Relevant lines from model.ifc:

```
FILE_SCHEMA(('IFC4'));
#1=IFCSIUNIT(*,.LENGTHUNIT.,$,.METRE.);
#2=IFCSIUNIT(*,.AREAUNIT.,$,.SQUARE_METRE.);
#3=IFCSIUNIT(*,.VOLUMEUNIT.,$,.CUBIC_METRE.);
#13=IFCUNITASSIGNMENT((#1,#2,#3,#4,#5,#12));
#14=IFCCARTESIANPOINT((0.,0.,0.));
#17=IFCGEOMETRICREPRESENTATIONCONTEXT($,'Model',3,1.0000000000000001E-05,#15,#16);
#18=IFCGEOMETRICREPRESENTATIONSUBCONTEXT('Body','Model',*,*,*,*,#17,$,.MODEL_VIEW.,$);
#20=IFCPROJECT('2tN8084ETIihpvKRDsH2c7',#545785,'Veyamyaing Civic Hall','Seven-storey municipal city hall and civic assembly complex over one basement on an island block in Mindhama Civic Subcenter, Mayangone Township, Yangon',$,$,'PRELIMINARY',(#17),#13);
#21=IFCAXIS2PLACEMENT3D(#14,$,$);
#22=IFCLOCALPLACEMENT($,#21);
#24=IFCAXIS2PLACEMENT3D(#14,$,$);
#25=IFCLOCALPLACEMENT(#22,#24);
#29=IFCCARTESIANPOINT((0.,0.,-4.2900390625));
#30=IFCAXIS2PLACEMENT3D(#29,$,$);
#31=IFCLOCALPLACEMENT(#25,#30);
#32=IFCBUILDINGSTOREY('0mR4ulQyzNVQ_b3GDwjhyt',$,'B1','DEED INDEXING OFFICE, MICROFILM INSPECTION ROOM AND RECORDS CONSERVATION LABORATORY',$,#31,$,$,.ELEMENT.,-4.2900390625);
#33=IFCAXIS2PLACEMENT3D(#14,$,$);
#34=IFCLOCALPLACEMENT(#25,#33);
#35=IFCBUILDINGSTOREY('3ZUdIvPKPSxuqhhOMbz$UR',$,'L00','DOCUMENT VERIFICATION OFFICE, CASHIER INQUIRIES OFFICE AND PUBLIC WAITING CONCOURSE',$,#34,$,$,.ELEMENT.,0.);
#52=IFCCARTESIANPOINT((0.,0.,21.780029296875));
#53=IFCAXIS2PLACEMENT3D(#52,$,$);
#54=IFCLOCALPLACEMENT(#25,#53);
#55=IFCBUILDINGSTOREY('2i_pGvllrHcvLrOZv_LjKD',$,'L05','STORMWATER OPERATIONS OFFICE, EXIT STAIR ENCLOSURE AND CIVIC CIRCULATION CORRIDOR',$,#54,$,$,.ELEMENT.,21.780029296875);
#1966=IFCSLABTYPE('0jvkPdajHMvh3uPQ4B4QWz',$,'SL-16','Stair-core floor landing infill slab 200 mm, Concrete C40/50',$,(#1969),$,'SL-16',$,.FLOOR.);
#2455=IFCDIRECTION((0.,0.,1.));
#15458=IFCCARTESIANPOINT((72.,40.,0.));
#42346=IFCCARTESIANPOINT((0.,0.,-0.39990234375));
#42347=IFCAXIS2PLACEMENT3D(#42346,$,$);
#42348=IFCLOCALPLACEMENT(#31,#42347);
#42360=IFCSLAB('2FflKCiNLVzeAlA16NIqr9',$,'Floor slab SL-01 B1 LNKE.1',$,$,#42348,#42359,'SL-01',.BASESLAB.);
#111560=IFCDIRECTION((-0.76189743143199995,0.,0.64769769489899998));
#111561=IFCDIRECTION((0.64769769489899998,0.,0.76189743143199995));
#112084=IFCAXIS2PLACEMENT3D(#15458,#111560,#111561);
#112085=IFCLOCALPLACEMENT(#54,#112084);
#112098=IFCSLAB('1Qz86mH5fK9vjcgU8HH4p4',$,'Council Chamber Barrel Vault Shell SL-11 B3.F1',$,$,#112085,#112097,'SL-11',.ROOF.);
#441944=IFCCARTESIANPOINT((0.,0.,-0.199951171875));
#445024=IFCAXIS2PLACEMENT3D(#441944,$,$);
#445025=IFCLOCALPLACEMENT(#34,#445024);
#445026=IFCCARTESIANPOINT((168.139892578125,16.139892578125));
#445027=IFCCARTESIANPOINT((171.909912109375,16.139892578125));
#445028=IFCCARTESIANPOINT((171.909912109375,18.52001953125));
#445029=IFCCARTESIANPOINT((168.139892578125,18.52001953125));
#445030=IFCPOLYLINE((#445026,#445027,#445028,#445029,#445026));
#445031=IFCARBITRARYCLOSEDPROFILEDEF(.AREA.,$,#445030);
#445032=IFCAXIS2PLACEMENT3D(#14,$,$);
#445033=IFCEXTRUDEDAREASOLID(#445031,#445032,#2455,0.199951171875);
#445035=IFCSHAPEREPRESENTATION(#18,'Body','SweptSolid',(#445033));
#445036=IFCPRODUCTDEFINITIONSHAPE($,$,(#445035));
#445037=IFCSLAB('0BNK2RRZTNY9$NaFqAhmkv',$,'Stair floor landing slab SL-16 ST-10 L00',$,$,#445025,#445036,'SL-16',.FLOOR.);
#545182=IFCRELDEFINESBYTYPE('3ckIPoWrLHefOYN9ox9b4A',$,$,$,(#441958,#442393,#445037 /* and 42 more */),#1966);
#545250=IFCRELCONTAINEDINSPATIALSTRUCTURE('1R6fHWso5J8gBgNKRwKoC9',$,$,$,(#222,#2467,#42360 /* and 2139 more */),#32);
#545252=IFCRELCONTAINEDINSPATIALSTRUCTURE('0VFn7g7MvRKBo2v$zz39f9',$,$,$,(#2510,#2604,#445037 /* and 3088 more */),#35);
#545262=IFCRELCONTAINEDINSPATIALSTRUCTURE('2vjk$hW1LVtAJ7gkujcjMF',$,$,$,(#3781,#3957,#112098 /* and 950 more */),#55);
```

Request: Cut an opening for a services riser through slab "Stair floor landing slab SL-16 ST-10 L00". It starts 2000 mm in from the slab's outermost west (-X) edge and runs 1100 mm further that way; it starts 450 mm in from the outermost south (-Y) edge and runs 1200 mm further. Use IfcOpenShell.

```python
import numpy as np
import ifcopenshell
import ifcopenshell.api.feature
import ifcopenshell.api.geometry
import ifcopenshell.api.root
import ifcopenshell.geom
import ifcopenshell.util.placement
import ifcopenshell.util.representation
import ifcopenshell.util.shape
import ifcopenshell.util.unit

model = ifcopenshell.open("model.ifc")
unit_scale = ifcopenshell.util.unit.calculate_unit_scale(model)
settings = ifcopenshell.geom.settings()


def volume(element):
    """Net volume in cubic metres, openings subtracted."""
    shape = ifcopenshell.geom.create_shape(settings, element)
    return ifcopenshell.util.shape.get_volume(shape.geometry)


slab = model.by_id(445037)
before = volume(slab)

# Extent in the slab's own axes, in metres. The edges named are its -X and -Y sides.
slab_shape = ifcopenshell.geom.create_shape(settings, slab)
vertices = ifcopenshell.util.shape.get_vertices(slab_shape.geometry)
x_min, y_min, bottom = vertices.min(axis=0)
top = vertices[:, 2].max()

opening = ifcopenshell.api.root.create_entity(model, ifc_class="IfcOpeningElement", name="Services riser opening", predefined_type="OPENING")
context = ifcopenshell.util.representation.get_context(model, "Model", "Body", "MODEL_VIEW")
width, depth = 1.1, 1.2
outline = [(0.0, 0.0), (width, 0.0), (width, depth), (0.0, depth), (0.0, 0.0)]
# Overshoot both faces by 50 mm so the cut is clean.
shape = ifcopenshell.api.geometry.add_slab_representation(
    model, context=context, depth=top - bottom + 0.1, polyline=outline
)
ifcopenshell.api.geometry.assign_representation(model, product=opening, representation=shape)

matrix = ifcopenshell.util.placement.get_local_placement(slab.ObjectPlacement)
matrix[:, 3] = matrix @ np.append(np.array([x_min + 2, y_min + 0.45, bottom - 0.05]) / unit_scale, 1.0)
ifcopenshell.api.geometry.edit_object_placement(model, product=opening, matrix=matrix, is_si=False)
ifcopenshell.api.feature.add_feature(model, feature=opening, element=slab)

after = volume(slab)

print(f"slab volume {before:.3f} -> {after:.3f} m3")

model.write("model_v2.ifc")
```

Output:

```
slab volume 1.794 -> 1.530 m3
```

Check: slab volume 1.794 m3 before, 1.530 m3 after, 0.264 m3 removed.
